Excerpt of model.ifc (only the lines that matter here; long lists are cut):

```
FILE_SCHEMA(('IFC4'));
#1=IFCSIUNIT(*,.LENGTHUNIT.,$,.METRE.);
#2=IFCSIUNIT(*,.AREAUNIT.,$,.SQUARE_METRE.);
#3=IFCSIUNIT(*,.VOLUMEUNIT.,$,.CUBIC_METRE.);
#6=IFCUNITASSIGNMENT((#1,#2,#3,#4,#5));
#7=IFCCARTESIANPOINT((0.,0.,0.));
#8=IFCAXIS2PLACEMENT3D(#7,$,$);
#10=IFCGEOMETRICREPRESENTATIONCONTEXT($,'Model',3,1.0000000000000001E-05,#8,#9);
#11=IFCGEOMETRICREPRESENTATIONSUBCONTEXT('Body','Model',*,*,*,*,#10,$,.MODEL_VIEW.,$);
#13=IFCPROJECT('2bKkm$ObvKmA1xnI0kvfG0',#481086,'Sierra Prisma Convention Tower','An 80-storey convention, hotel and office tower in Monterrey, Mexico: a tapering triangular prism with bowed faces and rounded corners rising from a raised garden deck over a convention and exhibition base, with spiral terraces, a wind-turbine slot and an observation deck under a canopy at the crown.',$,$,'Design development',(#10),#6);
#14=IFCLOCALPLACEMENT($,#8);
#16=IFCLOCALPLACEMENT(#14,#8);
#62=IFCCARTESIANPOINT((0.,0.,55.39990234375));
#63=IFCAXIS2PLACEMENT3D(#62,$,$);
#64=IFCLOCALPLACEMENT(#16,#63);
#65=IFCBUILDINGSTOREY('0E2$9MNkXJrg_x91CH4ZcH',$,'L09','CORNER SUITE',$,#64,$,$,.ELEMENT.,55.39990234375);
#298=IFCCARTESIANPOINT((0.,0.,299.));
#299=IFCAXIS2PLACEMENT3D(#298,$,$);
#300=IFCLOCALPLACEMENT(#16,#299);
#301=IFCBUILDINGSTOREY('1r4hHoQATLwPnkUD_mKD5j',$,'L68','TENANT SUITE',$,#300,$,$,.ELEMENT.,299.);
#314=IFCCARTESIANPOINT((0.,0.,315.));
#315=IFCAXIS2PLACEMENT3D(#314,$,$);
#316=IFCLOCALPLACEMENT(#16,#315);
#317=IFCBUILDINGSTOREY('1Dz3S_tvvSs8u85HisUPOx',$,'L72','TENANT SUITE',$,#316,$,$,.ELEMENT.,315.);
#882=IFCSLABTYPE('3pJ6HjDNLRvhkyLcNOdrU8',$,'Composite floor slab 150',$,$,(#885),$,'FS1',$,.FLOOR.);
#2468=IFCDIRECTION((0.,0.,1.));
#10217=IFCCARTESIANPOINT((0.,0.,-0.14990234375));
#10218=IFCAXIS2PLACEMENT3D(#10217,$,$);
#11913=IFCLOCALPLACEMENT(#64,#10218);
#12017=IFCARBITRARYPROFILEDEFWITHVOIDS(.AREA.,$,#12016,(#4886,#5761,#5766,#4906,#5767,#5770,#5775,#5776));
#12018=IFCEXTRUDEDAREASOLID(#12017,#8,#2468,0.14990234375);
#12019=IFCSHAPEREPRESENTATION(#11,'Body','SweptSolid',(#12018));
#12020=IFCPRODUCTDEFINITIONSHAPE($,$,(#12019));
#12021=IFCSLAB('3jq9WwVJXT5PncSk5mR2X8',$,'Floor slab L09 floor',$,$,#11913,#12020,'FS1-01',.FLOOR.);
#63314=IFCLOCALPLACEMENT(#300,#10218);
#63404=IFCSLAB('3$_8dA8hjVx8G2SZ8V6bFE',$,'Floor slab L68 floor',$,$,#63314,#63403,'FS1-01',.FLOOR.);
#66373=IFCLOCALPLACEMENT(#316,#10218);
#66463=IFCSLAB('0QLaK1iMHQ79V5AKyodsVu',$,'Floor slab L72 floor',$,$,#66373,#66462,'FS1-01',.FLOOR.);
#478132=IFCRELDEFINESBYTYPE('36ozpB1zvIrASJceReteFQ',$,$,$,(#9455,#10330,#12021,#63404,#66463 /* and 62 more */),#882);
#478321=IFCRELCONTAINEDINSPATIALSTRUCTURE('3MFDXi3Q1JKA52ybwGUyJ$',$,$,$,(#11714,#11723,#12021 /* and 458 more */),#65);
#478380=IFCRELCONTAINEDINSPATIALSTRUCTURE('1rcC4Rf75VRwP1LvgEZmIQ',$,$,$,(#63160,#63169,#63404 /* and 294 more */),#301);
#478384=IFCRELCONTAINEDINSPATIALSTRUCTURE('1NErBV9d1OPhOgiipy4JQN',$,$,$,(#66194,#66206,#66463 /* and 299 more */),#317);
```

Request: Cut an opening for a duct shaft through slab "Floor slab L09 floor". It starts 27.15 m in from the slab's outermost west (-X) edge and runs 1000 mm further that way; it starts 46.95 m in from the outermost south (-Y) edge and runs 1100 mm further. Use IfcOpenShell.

```python
import numpy as np
import ifcopenshell
import ifcopenshell.api.feature
import ifcopenshell.api.geometry
import ifcopenshell.api.root
import ifcopenshell.geom
import ifcopenshell.util.placement
import ifcopenshell.util.representation
import ifcopenshell.util.shape
import ifcopenshell.util.unit

model = ifcopenshell.open("model.ifc")
unit_scale = ifcopenshell.util.unit.calculate_unit_scale(model)
settings = ifcopenshell.geom.settings()


def volume(element):
    """Net volume in cubic metres, openings subtracted."""
    shape = ifcopenshell.geom.create_shape(settings, element)
    return ifcopenshell.util.shape.get_volume(shape.geometry)


slab = model.by_guid("3jq9WwVJXT5PncSk5mR2X8")
before = volume(slab)

# Extent in the slab's own axes, in metres. The edges named are its -X and -Y sides.
slab_shape = ifcopenshell.geom.create_shape(settings, slab)
vertices = ifcopenshell.util.shape.get_vertices(slab_shape.geometry)
x_min, y_min, bottom = vertices.min(axis=0)
top = vertices[:, 2].max()

opening = ifcopenshell.api.root.create_entity(model, ifc_class="IfcOpeningElement", name="Duct shaft opening", predefined_type="OPENING")
context = ifcopenshell.util.representation.get_context(model, "Model", "Body", "MODEL_VIEW")
width, depth = 1, 1.1
outline = [(0.0, 0.0), (width, 0.0), (width, depth), (0.0, depth), (0.0, 0.0)]
# Overshoot both faces by 50 mm so the cut is clean.
shape = ifcopenshell.api.geometry.add_slab_representation(
    model, context=context, depth=top - bottom + 0.1, polyline=outline
)
ifcopenshell.api.geometry.assign_representation(model, product=opening, representation=shape)

matrix = ifcopenshell.util.placement.get_local_placement(slab.ObjectPlacement)
matrix[:, 3] = matrix @ np.append(np.array([x_min + 27.15, y_min + 46.95, bottom - 0.05]) / unit_scale, 1.0)
ifcopenshell.api.geometry.edit_object_placement(model, product=opening, matrix=matrix, is_si=False)
ifcopenshell.api.feature.add_feature(model, feature=opening, element=slab)

after = volume(slab)

print(f"slab volume {before:.3f} -> {after:.3f} m3")

model.write("model_rev.ifc")
```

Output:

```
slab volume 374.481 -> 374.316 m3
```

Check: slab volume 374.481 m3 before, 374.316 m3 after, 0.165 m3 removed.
